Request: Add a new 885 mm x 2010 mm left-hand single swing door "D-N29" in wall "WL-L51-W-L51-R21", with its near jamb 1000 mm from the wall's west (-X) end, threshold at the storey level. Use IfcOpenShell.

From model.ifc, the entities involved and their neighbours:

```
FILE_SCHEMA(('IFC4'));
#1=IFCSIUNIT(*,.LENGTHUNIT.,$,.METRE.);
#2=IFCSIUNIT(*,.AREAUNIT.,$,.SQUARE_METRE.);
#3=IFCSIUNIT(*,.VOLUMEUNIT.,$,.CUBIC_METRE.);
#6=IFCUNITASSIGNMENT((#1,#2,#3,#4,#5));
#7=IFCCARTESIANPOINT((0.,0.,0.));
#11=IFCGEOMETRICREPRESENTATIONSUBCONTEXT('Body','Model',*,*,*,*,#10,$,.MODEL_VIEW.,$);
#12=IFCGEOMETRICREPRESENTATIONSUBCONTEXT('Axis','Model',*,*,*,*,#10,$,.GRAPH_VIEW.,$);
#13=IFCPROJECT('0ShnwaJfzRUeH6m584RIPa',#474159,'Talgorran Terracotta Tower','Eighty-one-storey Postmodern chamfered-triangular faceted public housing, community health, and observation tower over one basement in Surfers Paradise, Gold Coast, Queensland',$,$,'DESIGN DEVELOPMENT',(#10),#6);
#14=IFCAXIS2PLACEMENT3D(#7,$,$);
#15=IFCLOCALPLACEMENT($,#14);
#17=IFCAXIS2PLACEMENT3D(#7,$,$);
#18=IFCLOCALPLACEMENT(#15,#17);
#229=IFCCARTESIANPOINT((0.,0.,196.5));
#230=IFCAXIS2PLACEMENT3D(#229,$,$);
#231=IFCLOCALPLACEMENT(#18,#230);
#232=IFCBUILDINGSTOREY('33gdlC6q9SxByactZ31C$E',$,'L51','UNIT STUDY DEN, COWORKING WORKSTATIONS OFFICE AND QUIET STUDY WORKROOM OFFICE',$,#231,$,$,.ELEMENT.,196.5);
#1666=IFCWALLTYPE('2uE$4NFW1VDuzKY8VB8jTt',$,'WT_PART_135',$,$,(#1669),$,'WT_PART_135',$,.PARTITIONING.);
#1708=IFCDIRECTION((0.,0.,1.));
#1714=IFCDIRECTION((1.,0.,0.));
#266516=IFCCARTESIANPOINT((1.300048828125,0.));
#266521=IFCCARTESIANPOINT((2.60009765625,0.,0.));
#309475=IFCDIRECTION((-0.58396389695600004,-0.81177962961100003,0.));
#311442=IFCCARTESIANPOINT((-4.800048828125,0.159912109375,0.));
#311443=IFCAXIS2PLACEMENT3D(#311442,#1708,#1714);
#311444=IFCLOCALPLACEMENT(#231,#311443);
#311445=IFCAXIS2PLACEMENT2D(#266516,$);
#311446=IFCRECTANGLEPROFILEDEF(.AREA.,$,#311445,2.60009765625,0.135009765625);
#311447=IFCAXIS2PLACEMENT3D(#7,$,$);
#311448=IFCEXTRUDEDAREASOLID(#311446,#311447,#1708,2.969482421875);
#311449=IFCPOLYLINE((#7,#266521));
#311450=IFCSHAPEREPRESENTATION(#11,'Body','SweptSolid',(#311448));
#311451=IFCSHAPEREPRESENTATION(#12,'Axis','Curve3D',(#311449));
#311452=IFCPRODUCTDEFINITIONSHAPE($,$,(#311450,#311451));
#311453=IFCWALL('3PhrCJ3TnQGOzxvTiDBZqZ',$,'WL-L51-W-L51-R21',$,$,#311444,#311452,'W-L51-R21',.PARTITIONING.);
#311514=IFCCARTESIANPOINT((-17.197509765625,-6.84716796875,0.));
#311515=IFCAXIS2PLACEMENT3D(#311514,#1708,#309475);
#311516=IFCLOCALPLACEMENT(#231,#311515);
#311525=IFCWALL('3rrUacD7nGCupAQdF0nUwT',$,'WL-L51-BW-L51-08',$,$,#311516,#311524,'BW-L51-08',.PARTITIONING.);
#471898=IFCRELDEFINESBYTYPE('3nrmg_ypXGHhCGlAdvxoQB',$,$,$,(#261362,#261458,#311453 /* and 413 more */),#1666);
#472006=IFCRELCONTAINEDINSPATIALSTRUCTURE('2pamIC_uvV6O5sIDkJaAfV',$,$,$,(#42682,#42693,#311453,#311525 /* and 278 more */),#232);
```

```python
import numpy as np
import ifcopenshell
import ifcopenshell.api.feature
import ifcopenshell.api.geometry
import ifcopenshell.api.root
import ifcopenshell.api.spatial
import ifcopenshell.geom
import ifcopenshell.util.element
import ifcopenshell.util.placement
import ifcopenshell.util.representation
import ifcopenshell.util.shape
import ifcopenshell.util.unit

model = ifcopenshell.open("model.ifc")
unit_scale = ifcopenshell.util.unit.calculate_unit_scale(model)
settings = ifcopenshell.geom.settings()


def volume(element):
    """Net volume in cubic metres, openings subtracted."""
    shape = ifcopenshell.geom.create_shape(settings, element)
    return ifcopenshell.util.shape.get_volume(shape.geometry)


wall = model.by_id(311453)
storey = ifcopenshell.util.element.get_container(wall, ifc_class="IfcBuildingStorey")
context = ifcopenshell.util.representation.get_context(model, "Model", "Body", "MODEL_VIEW")
before = volume(wall)

width, height, from_end, sill = 0.885, 2.01, 1, 0.0  # metres

# The wall runs along its own X axis, and the end named is its -X end.
wall_shape = ifcopenshell.geom.create_shape(settings, wall)
x, y, z = ifcopenshell.util.shape.get_vertices(wall_shape.geometry).T
start = x.min() + from_end
face, thickness = float(y.min()), float(y.max() - y.min())
wall_matrix = ifcopenshell.util.placement.get_local_placement(wall.ObjectPlacement)
level = ifcopenshell.util.placement.get_local_placement(storey.ObjectPlacement)[2, 3]


def in_wall(x, y):
    """Placement at x, y metres in the wall's axes, at sill height."""
    matrix = wall_matrix.copy()
    matrix[:, 3] = wall_matrix @ np.array([x / unit_scale, y / unit_scale, 0.0, 1.0])
    matrix[2, 3] = level + sill / unit_scale
    return matrix


# Opening: a box that overshoots both wall faces by 50 mm.
opening = ifcopenshell.api.root.create_entity(model, ifc_class="IfcOpeningElement", predefined_type="OPENING")
box = ifcopenshell.api.geometry.add_wall_representation(
    model, context=context, length=width, height=height, thickness=thickness + 0.1
)
ifcopenshell.api.geometry.assign_representation(model, product=opening, representation=box)
ifcopenshell.api.geometry.edit_object_placement(model, product=opening, matrix=in_wall(start, face - 0.05), is_si=False)
ifcopenshell.api.feature.add_feature(model, feature=opening, element=wall)

door = ifcopenshell.api.root.create_entity(model, ifc_class="IfcDoor", name="D-N29", predefined_type="DOOR")
door.OverallWidth, door.OverallHeight = width / unit_scale, height / unit_scale
door.OperationType = "SINGLE_SWING_LEFT"
body = ifcopenshell.api.geometry.add_door_representation(
    model,
    context=context,
    overall_width=door.OverallWidth,
    overall_height=door.OverallHeight,
    operation_type="SINGLE_SWING_LEFT",
    lining_properties={"LiningDepth": thickness / unit_scale, "ThresholdDepth": thickness / unit_scale},
)
ifcopenshell.api.geometry.assign_representation(model, product=door, representation=body)
ifcopenshell.api.spatial.assign_container(model, products=[door], relating_structure=storey)
ifcopenshell.api.feature.add_filling(model, opening=opening, element=door)

# The lining spans the wall, so the door starts at the wall face.
ifcopenshell.api.geometry.edit_object_placement(model, product=door, matrix=in_wall(start, face), is_si=False)

after = volume(wall)

print(f"wall volume {before:.3f} -> {after:.3f} m3")

model.write("model_v2.ifc")
```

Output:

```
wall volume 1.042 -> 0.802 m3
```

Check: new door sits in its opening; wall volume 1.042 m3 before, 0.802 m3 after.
